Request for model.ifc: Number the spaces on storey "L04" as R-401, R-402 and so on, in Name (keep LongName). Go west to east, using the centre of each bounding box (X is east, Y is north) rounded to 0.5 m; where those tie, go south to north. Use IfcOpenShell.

First a look at what the model holds.

```python
import ifcopenshell
import ifcopenshell.util.element
import ifcopenshell.util.placement

model = ifcopenshell.open("model.ifc")
print(model.schema)
storey = next(s for s in model.by_type("IfcBuildingStorey") if s.Name == "L04")
spaces = [e for e in ifcopenshell.util.element.get_decomposition(storey) if e.is_a("IfcSpace")]
for e in sorted(spaces, key=lambda e: e.id()):
    origin = ifcopenshell.util.placement.get_local_placement(e.ObjectPlacement)[:3, 3]
    print(e.id(), e.Name, e.LongName, origin.round(2) + 0.0, sep=" | ")
```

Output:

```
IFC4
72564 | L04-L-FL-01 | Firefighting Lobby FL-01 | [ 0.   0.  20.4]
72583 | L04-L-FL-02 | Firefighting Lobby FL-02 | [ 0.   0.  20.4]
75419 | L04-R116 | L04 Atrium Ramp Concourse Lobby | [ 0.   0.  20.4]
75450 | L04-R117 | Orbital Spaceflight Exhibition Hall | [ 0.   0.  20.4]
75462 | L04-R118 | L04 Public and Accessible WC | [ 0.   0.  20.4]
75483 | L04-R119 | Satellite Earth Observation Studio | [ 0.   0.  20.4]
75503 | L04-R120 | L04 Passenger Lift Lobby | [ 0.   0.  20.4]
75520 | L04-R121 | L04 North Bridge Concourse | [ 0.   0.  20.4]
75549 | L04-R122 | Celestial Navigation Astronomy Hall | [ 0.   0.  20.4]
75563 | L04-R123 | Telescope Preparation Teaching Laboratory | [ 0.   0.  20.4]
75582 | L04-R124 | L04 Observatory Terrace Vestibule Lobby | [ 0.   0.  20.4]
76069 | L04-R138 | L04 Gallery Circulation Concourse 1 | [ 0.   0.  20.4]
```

```python
import ifcopenshell
import ifcopenshell.geom
import ifcopenshell.util.element
import ifcopenshell.util.shape

model = ifcopenshell.open("model.ifc")
settings = ifcopenshell.geom.settings()
settings.set("use-world-coords", True)


def centre(element):
    shape = ifcopenshell.geom.create_shape(settings, element)
    return ifcopenshell.util.shape.get_bbox_centroid(shape.geometry)


storey = next(s for s in model.by_type("IfcBuildingStorey") if s.Name == "L04")
spaces = [e for e in ifcopenshell.util.element.get_decomposition(storey) if e.is_a("IfcSpace")]

# Insertion points can sit at a corner or the storey origin, so sort by the geometry (in metres).
centres = {e: centre(e) for e in spaces}
spaces.sort(key=lambda e: (round(centres[e][0] / 0.5), centres[e][1]))

for i, e in enumerate(spaces, start=1):
    number = f"R-4{i:02d}"
    e.Name = number
    print(e.id(), number)

model.write("model_updated.ifc")
```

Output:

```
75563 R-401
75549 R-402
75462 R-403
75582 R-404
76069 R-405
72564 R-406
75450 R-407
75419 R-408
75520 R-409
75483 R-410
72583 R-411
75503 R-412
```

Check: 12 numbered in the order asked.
